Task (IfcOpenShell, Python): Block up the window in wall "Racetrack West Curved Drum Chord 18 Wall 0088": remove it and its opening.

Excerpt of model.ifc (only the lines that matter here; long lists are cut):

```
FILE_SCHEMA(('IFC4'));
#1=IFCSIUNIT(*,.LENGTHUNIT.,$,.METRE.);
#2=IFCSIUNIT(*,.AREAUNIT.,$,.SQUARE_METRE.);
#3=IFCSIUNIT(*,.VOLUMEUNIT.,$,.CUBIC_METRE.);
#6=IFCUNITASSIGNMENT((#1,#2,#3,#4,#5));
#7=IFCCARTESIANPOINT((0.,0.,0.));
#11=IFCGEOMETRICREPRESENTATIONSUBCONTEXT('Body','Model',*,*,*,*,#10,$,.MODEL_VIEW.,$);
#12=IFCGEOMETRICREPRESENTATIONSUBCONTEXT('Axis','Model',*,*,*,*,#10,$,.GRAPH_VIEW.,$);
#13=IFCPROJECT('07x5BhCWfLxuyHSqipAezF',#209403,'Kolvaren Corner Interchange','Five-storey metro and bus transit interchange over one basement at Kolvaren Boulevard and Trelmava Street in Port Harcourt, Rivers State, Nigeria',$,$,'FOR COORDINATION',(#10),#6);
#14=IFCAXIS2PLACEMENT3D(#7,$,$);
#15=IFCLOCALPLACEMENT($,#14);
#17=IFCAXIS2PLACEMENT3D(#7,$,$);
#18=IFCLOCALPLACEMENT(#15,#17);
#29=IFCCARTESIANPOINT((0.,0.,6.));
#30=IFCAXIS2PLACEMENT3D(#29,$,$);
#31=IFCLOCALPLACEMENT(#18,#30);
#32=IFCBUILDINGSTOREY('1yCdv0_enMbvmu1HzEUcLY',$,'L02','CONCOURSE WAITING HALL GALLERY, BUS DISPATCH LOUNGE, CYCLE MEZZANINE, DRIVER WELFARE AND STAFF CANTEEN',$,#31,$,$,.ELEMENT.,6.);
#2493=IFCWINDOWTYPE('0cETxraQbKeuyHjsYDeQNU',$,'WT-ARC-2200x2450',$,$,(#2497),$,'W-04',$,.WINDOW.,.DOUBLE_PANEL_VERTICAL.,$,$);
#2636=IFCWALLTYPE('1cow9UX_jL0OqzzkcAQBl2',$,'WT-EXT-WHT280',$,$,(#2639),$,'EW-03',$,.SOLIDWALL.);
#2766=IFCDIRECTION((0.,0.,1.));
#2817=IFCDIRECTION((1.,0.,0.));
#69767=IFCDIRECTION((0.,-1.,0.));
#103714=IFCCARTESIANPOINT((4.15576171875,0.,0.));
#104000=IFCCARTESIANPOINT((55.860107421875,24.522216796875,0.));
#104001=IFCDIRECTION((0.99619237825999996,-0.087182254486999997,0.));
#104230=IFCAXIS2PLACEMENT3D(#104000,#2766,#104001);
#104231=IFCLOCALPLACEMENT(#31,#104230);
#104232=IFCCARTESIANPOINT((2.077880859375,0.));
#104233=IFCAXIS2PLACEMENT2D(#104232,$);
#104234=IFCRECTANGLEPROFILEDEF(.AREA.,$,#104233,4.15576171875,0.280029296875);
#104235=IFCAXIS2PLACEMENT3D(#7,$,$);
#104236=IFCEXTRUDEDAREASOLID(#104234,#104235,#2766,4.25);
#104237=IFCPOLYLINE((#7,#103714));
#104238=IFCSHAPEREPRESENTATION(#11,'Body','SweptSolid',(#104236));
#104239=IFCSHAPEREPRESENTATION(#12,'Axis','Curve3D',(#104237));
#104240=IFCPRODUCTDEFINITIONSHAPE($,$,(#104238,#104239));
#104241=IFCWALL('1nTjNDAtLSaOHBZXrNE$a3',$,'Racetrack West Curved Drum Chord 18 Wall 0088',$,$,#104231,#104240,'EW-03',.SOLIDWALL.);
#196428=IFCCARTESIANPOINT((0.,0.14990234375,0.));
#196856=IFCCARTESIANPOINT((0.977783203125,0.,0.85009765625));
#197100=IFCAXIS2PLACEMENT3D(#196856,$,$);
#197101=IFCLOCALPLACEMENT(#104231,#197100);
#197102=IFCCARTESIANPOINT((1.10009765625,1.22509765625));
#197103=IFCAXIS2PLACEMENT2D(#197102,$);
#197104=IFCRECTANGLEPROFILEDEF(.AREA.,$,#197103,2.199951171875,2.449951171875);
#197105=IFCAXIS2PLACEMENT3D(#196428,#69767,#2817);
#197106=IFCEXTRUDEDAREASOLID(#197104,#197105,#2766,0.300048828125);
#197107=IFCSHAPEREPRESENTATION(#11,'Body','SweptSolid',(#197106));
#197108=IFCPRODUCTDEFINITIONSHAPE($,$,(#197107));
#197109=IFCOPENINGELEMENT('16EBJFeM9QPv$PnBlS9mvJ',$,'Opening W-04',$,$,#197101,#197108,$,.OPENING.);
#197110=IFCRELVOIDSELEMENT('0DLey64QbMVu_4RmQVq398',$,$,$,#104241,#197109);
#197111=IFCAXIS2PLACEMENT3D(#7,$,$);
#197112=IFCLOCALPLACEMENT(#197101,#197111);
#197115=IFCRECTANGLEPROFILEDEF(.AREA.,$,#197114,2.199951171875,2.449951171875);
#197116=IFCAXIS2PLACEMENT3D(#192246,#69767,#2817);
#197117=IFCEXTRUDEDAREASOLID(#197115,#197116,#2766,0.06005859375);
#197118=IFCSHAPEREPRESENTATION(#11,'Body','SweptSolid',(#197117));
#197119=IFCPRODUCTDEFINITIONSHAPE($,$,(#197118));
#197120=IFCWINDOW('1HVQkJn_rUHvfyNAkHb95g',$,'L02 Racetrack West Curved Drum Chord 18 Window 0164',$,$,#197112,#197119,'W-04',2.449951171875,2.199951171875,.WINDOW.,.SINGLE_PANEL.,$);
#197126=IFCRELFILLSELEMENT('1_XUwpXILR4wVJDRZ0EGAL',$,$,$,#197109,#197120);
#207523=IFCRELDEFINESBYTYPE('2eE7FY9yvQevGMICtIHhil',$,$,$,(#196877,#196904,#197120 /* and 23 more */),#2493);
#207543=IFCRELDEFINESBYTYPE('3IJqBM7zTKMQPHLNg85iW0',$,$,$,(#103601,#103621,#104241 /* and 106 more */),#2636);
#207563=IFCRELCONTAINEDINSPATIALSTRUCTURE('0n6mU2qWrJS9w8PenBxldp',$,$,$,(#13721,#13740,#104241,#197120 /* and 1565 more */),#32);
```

```python
import ifcopenshell
import ifcopenshell.api.feature
import ifcopenshell.api.root
import ifcopenshell.geom
import ifcopenshell.util.shape

model = ifcopenshell.open("model.ifc")
settings = ifcopenshell.geom.settings()


def volume(element):
    """Net volume in cubic metres, openings subtracted."""
    shape = ifcopenshell.geom.create_shape(settings, element)
    return ifcopenshell.util.shape.get_volume(shape.geometry)


window = model.by_guid("1HVQkJn_rUHvfyNAkHb95g")
opening = window.FillsVoids[0].RelatingOpeningElement
wall = opening.VoidsElements[0].RelatingBuildingElement
before = volume(wall)

ifcopenshell.api.root.remove_product(model, product=window)
ifcopenshell.api.feature.remove_feature(model, feature=opening)

after = volume(wall)

print(f"wall volume {before:.3f} -> {after:.3f} m3")

model.write("model_updated.ifc")
```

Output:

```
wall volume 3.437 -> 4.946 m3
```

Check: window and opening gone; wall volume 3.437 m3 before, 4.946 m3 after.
